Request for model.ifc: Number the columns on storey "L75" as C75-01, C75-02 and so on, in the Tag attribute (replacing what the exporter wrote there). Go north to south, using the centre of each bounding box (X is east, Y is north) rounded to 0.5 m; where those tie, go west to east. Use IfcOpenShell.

First a look at what the model holds.

```python
import ifcopenshell
import ifcopenshell.util.element
import ifcopenshell.util.placement

model = ifcopenshell.open("model.ifc")
print(model.schema)
storey = next(s for s in model.by_type("IfcBuildingStorey") if s.Name == "L75")
columns = [e for e in ifcopenshell.util.element.get_decomposition(storey) if e.is_a("IfcColumn")]
for e in sorted(columns, key=lambda e: e.id()):
    origin = ifcopenshell.util.placement.get_local_placement(e.ObjectPlacement)[:3, 3]
    print(e.id(), e.Tag, e.Name, origin.round(2) + 0.0, sep=" | ")
```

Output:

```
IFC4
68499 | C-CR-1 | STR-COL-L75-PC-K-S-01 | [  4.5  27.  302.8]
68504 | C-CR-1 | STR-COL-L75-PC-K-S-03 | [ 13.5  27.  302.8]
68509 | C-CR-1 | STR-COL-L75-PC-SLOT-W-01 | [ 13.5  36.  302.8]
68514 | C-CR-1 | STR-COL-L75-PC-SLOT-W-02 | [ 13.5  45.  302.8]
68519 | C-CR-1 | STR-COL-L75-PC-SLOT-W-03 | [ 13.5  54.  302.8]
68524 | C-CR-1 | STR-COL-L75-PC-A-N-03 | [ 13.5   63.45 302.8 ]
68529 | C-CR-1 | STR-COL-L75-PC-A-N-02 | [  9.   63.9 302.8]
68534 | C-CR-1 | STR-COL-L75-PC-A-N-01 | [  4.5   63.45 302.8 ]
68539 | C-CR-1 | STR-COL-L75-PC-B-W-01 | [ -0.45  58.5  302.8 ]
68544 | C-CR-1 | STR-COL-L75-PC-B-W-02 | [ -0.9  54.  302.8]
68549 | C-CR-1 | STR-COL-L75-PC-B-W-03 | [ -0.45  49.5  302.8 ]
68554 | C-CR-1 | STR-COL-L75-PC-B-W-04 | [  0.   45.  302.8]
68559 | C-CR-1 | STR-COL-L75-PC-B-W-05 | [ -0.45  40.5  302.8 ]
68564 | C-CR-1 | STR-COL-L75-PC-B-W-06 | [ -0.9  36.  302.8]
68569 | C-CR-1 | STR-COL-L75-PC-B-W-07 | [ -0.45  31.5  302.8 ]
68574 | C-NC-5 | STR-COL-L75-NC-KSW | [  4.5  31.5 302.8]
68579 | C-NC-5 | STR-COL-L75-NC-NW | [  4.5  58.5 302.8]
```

```python
import ifcopenshell
import ifcopenshell.geom
import ifcopenshell.util.element
import ifcopenshell.util.shape

model = ifcopenshell.open("model.ifc")
settings = ifcopenshell.geom.settings()
settings.set("use-world-coords", True)


def centre(element):
    shape = ifcopenshell.geom.create_shape(settings, element)
    return ifcopenshell.util.shape.get_bbox_centroid(shape.geometry)


storey = next(s for s in model.by_type("IfcBuildingStorey") if s.Name == "L75")
columns = [e for e in ifcopenshell.util.element.get_decomposition(storey) if e.is_a("IfcColumn")]

# Insertion points can sit at a corner or the storey origin, so sort by the geometry (in metres).
centres = {e: centre(e) for e in columns}
columns.sort(key=lambda e: (-round(centres[e][1] / 0.5), centres[e][0]))

for i, e in enumerate(columns, start=1):
    number = f"C75-{i:02d}"
    e.Tag = number
    print(e.id(), number)

model.write("model-out.ifc")
```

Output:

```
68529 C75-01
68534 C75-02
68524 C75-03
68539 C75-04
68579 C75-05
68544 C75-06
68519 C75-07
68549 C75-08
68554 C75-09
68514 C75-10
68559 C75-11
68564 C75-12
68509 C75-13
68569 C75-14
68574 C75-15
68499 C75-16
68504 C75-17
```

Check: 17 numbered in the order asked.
